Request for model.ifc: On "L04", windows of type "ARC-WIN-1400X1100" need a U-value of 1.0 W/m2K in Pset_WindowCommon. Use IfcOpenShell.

First a look at what the model holds.

```python
import ifcopenshell
import ifcopenshell.util.element

model = ifcopenshell.open("model.ifc")
print(model.schema)
storey = next(s for s in model.by_type("IfcBuildingStorey") if s.Name == "L04")
windows = [e for e in ifcopenshell.util.element.get_decomposition(storey) if e.is_a("IfcWindow")]
seen = {}
for e in windows:
    element_type = ifcopenshell.util.element.get_type(e)
    key = (element_type.Name if element_type != e and element_type else None, ifcopenshell.util.element.get_pset(e, "Pset_WindowCommon", "ThermalTransmittance"))
    seen[key] = seen.get(key, 0) + 1
for (name, value), count in sorted(seen.items(), key=str):
    print(count, "x", name, "|", value)
```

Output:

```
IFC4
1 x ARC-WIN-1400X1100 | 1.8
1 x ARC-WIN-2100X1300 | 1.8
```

```python
import ifcopenshell
import ifcopenshell.api.pset
import ifcopenshell.util.element

model = ifcopenshell.open("model.ifc")

storey = next(s for s in model.by_type("IfcBuildingStorey") if s.Name == "L04")
windows = [e for e in ifcopenshell.util.element.get_decomposition(storey) if e.is_a("IfcWindow")]

count = 0
for e in windows:
    element_type = ifcopenshell.util.element.get_type(e)
    if element_type in (None, e) or element_type.Name != "ARC-WIN-1400X1100":
        continue
    # add_pset returns the element's existing set when there is one.
    pset = ifcopenshell.api.pset.add_pset(model, product=e, name="Pset_WindowCommon")
    ifcopenshell.api.pset.edit_pset(model, pset=pset, properties={"ThermalTransmittance": 1.0})
    count += 1

print(count, "windows updated")

model.write("model-out.ifc")
```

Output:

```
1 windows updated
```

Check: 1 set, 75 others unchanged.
